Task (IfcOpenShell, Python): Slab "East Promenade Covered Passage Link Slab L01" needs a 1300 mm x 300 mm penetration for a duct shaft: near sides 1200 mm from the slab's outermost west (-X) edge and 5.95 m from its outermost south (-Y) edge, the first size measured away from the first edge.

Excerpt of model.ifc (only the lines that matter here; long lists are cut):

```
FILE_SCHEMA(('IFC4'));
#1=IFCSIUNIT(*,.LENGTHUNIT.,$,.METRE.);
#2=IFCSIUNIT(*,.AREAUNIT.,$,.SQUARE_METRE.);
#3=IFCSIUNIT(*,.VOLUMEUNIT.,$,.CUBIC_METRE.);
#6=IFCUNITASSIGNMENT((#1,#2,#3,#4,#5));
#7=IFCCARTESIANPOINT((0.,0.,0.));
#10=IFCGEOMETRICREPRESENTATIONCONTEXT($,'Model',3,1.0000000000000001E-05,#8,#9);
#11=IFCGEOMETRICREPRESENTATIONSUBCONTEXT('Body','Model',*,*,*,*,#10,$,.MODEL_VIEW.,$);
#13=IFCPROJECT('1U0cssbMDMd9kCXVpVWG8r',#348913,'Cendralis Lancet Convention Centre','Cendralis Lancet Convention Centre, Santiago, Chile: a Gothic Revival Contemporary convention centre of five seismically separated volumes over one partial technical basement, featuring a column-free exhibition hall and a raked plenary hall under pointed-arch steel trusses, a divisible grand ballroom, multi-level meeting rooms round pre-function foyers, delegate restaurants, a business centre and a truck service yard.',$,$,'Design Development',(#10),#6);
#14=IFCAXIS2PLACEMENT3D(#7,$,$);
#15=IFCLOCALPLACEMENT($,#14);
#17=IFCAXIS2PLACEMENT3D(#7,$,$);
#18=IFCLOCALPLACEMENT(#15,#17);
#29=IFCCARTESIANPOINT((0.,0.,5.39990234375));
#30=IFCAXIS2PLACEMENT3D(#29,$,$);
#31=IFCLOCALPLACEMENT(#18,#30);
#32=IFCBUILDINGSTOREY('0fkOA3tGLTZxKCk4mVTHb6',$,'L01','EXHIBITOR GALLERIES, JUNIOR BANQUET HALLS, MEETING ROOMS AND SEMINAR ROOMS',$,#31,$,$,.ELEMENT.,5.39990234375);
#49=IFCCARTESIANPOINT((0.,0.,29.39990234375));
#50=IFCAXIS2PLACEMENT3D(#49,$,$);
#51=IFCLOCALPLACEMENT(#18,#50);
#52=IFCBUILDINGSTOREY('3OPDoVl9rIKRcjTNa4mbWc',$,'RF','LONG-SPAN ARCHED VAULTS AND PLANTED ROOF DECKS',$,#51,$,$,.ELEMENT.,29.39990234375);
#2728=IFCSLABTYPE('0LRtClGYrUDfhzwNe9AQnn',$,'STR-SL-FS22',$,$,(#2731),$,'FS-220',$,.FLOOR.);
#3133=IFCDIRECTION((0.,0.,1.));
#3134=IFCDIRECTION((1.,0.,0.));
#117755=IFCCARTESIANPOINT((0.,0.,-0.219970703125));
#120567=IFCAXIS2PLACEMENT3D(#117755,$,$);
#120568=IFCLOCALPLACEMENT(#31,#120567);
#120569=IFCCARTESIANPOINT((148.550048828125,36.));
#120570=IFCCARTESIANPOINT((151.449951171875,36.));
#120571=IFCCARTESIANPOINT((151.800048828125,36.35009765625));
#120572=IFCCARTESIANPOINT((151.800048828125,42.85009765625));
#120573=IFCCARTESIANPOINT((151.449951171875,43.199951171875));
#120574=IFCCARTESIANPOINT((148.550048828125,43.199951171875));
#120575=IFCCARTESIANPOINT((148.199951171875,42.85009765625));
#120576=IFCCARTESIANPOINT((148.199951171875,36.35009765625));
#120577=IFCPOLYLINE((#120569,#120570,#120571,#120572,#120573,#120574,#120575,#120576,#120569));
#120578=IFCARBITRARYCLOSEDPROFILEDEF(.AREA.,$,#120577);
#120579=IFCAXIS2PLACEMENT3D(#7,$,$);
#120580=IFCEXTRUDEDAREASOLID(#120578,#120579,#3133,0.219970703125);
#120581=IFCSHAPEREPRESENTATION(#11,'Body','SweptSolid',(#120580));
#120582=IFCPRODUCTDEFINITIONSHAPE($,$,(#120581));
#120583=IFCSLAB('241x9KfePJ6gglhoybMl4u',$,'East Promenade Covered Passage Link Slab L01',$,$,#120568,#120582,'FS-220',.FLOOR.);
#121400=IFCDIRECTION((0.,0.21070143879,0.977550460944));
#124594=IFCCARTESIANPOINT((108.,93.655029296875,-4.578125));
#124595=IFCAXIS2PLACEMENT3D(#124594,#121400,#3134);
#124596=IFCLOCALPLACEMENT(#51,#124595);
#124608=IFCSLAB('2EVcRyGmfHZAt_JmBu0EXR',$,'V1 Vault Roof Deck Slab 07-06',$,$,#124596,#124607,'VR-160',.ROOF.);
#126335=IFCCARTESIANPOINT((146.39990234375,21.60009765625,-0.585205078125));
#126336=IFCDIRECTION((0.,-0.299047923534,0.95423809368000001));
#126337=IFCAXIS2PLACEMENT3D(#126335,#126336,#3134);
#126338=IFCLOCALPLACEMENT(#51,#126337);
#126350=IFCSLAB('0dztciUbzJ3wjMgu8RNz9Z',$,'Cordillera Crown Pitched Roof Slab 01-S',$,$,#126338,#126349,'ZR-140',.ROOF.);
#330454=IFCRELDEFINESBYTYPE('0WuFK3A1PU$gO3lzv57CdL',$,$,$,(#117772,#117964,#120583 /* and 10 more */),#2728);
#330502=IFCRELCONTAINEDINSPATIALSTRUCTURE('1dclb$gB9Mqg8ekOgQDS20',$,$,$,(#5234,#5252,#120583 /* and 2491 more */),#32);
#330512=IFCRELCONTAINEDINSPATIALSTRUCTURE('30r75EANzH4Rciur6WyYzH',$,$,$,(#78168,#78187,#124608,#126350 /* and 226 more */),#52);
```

```python
import numpy as np
import ifcopenshell
import ifcopenshell.api.feature
import ifcopenshell.api.geometry
import ifcopenshell.api.root
import ifcopenshell.geom
import ifcopenshell.util.placement
import ifcopenshell.util.representation
import ifcopenshell.util.shape
import ifcopenshell.util.unit

model = ifcopenshell.open("model.ifc")
unit_scale = ifcopenshell.util.unit.calculate_unit_scale(model)
settings = ifcopenshell.geom.settings()


def volume(element):
    """Net volume in cubic metres, openings subtracted."""
    shape = ifcopenshell.geom.create_shape(settings, element)
    return ifcopenshell.util.shape.get_volume(shape.geometry)


slab = model.by_guid("241x9KfePJ6gglhoybMl4u")
before = volume(slab)

# Extent in the slab's own axes, in metres. The edges named are its -X and -Y sides.
slab_shape = ifcopenshell.geom.create_shape(settings, slab)
vertices = ifcopenshell.util.shape.get_vertices(slab_shape.geometry)
x_min, y_min, bottom = vertices.min(axis=0)
top = vertices[:, 2].max()

opening = ifcopenshell.api.root.create_entity(model, ifc_class="IfcOpeningElement", name="Duct shaft opening", predefined_type="OPENING")
context = ifcopenshell.util.representation.get_context(model, "Model", "Body", "MODEL_VIEW")
width, depth = 1.3, 0.3
outline = [(0.0, 0.0), (width, 0.0), (width, depth), (0.0, depth), (0.0, 0.0)]
# Overshoot both faces by 50 mm so the cut is clean.
shape = ifcopenshell.api.geometry.add_slab_representation(
    model, context=context, depth=top - bottom + 0.1, polyline=outline
)
ifcopenshell.api.geometry.assign_representation(model, product=opening, representation=shape)

matrix = ifcopenshell.util.placement.get_local_placement(slab.ObjectPlacement)
matrix[:, 3] = matrix @ np.append(np.array([x_min + 1.2, y_min + 5.95, bottom - 0.05]) / unit_scale, 1.0)
ifcopenshell.api.geometry.edit_object_placement(model, product=opening, matrix=matrix, is_si=False)
ifcopenshell.api.feature.add_feature(model, feature=opening, element=slab)

after = volume(slab)

print(f"slab volume {before:.3f} -> {after:.3f} m3")

model.write("model_edited.ifc")
```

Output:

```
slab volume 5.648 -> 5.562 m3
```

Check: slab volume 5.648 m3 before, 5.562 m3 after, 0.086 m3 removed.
